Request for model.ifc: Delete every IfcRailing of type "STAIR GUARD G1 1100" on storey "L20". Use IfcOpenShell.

First a look at what the model holds.

```python
import ifcopenshell
import ifcopenshell.util.element

model = ifcopenshell.open("model.ifc")
print(model.schema)
storey = next(s for s in model.by_type("IfcBuildingStorey") if s.Name == "L20")
railings = [e for e in ifcopenshell.util.element.get_decomposition(storey) if e.is_a("IfcRailing")]
seen = {}
for e in railings:
    element_type = ifcopenshell.util.element.get_type(e)
    name = element_type.Name if element_type not in (None, e) else None
    seen[name] = seen.get(name, 0) + 1
for name, count in sorted(seen.items(), key=str):
    print(count, "x", name)
```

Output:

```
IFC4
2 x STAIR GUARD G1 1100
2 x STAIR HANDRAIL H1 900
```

```python
import ifcopenshell
import ifcopenshell.api.root
import ifcopenshell.util.element

model = ifcopenshell.open("model.ifc")

storey = next(s for s in model.by_type("IfcBuildingStorey") if s.Name == "L20")
railings = [e for e in ifcopenshell.util.element.get_decomposition(storey) if e.is_a("IfcRailing")]
targets = [e for e in railings if (t := ifcopenshell.util.element.get_type(e)) not in (None, e) and t.Name == "STAIR GUARD G1 1100"]

for e in targets:
    ifcopenshell.api.root.remove_product(model, product=e)
print(len(targets), "removed")

model.write("model_updated.ifc")
```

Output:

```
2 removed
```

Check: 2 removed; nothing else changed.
